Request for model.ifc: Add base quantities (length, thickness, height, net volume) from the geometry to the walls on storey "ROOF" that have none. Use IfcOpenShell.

First a look at what the model holds.

```python
import ifcopenshell
import ifcopenshell.util.element
import ifcopenshell.util.unit

model = ifcopenshell.open("model.ifc")
print(model.schema)
for unit_type in ("LENGTHUNIT", "AREAUNIT", "VOLUMEUNIT"):
    print(unit_type, ifcopenshell.util.unit.calculate_unit_scale(model, unit_type))
storey = next(s for s in model.by_type("IfcBuildingStorey") if s.Name == "ROOF")
walls = [e for e in ifcopenshell.util.element.get_decomposition(storey) if e.is_a("IfcWall")]
for e in sorted(walls, key=lambda e: e.id()):
    print(e.id(), e.is_a(), e.Name, list(ifcopenshell.util.element.get_psets(e, qtos_only=True)), sep=" | ")
```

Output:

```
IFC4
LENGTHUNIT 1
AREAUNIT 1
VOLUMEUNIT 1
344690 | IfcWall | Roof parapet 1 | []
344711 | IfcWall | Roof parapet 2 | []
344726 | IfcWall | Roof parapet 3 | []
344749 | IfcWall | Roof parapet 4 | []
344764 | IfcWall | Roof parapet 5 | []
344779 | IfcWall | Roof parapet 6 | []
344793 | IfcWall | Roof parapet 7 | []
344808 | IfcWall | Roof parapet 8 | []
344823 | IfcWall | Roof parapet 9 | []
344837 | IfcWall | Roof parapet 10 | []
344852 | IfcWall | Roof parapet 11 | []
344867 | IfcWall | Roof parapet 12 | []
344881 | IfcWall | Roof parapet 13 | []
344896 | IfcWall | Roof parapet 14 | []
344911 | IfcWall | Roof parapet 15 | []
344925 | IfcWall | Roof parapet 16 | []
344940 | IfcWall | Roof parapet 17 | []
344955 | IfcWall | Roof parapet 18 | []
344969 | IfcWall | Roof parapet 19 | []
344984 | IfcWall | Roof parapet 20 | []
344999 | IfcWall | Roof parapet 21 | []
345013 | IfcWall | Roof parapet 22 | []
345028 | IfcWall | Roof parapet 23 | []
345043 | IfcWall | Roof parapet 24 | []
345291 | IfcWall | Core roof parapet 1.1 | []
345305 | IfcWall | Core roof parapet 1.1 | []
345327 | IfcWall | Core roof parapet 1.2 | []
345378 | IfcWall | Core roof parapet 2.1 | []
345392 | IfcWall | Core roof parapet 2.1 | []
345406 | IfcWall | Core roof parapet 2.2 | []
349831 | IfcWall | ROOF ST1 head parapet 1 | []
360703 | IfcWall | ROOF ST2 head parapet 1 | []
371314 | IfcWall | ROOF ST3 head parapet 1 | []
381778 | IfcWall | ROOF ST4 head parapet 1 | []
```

```python
import ifcopenshell
import ifcopenshell.api.pset
import ifcopenshell.geom
import ifcopenshell.util.element
import ifcopenshell.util.shape
import ifcopenshell.util.unit

model = ifcopenshell.open("model.ifc")
unit_scale = ifcopenshell.util.unit.calculate_unit_scale(model)
volume_scale = ifcopenshell.util.unit.calculate_unit_scale(model, "VOLUMEUNIT")
settings = ifcopenshell.geom.settings()

storey = next(s for s in model.by_type("IfcBuildingStorey") if s.Name == "ROOF")
walls = [e for e in ifcopenshell.util.element.get_decomposition(storey) if e.is_a("IfcWall")]

for e in sorted(walls, key=lambda e: e.id()):
    if ifcopenshell.util.element.get_psets(e, qtos_only=True, should_inherit=False):
        continue
    # Geometry comes back in metres, in the element's own axes.
    shape = ifcopenshell.geom.create_shape(settings, e)
    values = {
        "Length": ifcopenshell.util.shape.get_x(shape.geometry) / unit_scale,
        "Width": ifcopenshell.util.shape.get_y(shape.geometry) / unit_scale,
        "Height": ifcopenshell.util.shape.get_z(shape.geometry) / unit_scale,
        "NetVolume": ifcopenshell.util.shape.get_volume(shape.geometry) / volume_scale,
    }
    qto = ifcopenshell.api.pset.add_qto(model, product=e, name="Qto_WallBaseQuantities")
    ifcopenshell.api.pset.edit_qto(model, qto=qto, properties=values)
    print(e.id(), {k: round(v, 3) for k, v in values.items()})

model.write("model_rev.ifc")
```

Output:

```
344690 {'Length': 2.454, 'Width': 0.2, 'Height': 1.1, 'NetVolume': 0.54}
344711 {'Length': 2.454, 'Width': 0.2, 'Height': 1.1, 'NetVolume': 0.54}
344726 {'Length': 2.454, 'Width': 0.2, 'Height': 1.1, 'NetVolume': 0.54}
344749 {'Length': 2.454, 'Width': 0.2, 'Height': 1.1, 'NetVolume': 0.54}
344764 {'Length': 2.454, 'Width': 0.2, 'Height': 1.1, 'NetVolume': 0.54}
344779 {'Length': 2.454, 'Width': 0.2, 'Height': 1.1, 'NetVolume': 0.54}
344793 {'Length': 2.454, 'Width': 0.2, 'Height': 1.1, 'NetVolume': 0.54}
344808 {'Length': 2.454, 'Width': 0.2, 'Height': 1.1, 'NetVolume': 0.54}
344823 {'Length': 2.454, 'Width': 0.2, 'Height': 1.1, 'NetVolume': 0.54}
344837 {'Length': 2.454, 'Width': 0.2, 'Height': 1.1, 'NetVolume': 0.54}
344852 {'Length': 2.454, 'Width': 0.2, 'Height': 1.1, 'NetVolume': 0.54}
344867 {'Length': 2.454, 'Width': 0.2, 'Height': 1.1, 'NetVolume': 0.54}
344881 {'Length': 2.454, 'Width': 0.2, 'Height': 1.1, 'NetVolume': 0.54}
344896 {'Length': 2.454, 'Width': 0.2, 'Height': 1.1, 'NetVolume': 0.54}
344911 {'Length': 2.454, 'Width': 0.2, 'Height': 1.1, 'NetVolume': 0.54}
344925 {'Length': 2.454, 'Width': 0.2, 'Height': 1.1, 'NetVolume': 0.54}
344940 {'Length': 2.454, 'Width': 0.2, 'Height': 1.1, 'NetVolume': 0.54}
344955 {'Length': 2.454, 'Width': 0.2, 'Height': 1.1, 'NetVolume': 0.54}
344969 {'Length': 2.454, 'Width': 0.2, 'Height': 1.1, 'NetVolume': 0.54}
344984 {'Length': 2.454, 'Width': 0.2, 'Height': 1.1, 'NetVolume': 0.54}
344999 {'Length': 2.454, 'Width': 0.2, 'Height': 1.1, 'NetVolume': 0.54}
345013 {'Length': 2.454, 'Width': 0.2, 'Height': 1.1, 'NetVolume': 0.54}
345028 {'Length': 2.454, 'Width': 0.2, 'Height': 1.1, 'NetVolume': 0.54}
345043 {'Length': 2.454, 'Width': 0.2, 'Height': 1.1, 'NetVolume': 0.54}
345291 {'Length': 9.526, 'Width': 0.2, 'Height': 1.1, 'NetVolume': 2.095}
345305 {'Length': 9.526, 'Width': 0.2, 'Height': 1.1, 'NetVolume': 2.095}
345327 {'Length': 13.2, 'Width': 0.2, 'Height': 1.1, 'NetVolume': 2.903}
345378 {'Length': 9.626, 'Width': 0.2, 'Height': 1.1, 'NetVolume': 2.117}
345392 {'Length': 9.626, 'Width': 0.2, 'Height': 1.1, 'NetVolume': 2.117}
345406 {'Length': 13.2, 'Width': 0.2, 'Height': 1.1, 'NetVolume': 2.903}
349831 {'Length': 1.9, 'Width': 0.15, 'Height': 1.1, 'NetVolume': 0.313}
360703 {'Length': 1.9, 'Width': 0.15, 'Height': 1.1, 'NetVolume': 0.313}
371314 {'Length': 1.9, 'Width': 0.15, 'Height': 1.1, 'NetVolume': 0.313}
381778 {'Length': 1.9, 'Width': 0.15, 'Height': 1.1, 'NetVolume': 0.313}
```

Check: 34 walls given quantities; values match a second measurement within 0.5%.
